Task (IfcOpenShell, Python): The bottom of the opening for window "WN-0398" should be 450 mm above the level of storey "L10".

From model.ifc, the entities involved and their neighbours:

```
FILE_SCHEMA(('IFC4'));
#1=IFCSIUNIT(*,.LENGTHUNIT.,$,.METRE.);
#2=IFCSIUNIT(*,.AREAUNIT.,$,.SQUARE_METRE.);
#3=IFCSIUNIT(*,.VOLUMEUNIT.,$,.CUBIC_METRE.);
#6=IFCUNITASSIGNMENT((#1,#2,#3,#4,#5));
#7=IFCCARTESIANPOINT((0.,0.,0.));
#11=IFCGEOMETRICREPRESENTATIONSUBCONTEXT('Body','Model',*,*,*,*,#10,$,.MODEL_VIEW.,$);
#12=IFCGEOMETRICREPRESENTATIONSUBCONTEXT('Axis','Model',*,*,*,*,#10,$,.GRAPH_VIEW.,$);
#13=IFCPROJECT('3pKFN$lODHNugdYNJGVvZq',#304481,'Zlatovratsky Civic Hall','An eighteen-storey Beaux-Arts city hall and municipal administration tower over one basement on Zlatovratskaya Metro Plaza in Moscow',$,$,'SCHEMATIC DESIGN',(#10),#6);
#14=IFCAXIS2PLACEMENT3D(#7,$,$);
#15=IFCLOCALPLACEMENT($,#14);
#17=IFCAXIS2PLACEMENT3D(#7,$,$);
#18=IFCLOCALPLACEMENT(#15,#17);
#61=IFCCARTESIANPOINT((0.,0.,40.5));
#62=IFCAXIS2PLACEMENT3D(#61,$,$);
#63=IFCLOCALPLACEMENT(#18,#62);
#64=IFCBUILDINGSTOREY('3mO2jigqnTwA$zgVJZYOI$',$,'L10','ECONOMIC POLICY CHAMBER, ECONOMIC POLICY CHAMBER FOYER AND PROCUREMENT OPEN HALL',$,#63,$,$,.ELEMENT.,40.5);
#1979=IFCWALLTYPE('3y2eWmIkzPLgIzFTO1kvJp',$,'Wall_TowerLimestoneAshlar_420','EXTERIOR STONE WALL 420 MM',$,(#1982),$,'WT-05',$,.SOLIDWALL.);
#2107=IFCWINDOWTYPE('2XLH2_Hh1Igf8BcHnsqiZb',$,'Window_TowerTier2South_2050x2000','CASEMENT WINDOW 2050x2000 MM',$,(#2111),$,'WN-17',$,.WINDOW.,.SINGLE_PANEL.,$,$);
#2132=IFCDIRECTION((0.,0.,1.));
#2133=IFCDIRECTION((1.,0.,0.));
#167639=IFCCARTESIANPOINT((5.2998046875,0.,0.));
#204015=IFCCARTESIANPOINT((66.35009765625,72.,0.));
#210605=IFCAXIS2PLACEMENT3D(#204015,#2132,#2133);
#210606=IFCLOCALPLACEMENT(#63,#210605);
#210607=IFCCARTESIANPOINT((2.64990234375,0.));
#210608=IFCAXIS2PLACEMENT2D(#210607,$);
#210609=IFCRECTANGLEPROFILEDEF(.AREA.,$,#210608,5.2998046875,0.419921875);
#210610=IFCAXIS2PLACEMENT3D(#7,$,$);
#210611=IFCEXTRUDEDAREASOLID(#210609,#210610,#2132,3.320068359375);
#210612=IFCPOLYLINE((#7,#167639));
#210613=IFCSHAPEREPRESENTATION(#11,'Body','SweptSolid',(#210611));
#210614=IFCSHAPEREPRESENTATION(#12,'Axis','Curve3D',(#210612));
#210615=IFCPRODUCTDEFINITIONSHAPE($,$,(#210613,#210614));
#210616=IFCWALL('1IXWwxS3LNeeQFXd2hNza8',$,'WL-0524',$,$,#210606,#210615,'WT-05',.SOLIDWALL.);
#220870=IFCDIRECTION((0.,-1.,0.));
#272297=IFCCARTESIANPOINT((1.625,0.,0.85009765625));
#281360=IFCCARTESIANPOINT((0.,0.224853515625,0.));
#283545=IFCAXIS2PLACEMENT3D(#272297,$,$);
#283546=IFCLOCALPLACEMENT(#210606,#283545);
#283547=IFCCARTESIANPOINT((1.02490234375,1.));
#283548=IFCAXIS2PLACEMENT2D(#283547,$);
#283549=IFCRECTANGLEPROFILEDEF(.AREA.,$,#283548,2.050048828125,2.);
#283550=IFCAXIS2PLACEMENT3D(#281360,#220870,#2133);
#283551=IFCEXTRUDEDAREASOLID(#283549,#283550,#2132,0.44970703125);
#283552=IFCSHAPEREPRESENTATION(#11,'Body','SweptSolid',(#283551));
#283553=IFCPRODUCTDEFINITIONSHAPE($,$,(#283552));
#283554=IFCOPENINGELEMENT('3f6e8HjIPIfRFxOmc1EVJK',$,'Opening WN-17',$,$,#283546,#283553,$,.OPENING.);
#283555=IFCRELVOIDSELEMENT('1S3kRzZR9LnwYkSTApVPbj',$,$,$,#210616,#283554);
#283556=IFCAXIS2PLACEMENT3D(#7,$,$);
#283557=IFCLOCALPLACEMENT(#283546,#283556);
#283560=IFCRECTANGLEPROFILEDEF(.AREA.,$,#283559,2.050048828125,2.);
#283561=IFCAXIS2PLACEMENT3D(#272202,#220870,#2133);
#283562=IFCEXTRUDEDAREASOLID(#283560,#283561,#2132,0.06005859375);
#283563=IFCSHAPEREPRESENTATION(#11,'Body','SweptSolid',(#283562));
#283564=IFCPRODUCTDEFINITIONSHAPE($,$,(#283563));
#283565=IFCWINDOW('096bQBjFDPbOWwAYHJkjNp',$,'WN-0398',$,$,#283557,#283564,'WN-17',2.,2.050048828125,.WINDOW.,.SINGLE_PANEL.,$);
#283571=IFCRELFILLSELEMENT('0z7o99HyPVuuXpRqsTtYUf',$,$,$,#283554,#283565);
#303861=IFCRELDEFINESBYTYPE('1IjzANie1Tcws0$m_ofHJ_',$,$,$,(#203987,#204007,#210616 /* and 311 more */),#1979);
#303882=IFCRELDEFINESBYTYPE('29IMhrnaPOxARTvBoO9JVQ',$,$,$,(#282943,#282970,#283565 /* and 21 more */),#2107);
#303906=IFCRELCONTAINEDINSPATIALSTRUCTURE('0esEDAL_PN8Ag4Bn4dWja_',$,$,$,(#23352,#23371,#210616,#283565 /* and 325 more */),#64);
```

```python
import numpy as np
import ifcopenshell
import ifcopenshell.api.geometry
import ifcopenshell.geom
import ifcopenshell.util.element
import ifcopenshell.util.placement
import ifcopenshell.util.shape
import ifcopenshell.util.unit

model = ifcopenshell.open("model.ifc")
unit_scale = ifcopenshell.util.unit.calculate_unit_scale(model)

window = model.by_id(283565)
opening = window.FillsVoids[0].RelatingOpeningElement
storey = ifcopenshell.util.element.get_container(window, ifc_class="IfcBuildingStorey")
level = ifcopenshell.util.placement.get_local_placement(storey.ObjectPlacement)[2, 3]

# The opening's origin need not be at the sill, so measure its lowest point.
shape = ifcopenshell.geom.create_shape(ifcopenshell.geom.settings(), opening)
bottom = ifcopenshell.util.shape.get_shape_bottom_elevation(shape, shape.geometry) / unit_scale
dz = level + 0.45 / unit_scale - bottom

shift = np.array([0.0, 0.0, dz])
# The window is placed relative to its opening, so it follows when the opening moves.
matrix = ifcopenshell.util.placement.get_local_placement(opening.ObjectPlacement)
matrix[:3, 3] += shift
ifcopenshell.api.geometry.edit_object_placement(
    model, product=opening, matrix=matrix, is_si=False, should_transform_children=True
)

print(f"moved by {dz * unit_scale:+.3f} m")

model.write("model_edited.ifc")
```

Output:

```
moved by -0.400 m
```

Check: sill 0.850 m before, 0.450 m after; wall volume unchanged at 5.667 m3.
